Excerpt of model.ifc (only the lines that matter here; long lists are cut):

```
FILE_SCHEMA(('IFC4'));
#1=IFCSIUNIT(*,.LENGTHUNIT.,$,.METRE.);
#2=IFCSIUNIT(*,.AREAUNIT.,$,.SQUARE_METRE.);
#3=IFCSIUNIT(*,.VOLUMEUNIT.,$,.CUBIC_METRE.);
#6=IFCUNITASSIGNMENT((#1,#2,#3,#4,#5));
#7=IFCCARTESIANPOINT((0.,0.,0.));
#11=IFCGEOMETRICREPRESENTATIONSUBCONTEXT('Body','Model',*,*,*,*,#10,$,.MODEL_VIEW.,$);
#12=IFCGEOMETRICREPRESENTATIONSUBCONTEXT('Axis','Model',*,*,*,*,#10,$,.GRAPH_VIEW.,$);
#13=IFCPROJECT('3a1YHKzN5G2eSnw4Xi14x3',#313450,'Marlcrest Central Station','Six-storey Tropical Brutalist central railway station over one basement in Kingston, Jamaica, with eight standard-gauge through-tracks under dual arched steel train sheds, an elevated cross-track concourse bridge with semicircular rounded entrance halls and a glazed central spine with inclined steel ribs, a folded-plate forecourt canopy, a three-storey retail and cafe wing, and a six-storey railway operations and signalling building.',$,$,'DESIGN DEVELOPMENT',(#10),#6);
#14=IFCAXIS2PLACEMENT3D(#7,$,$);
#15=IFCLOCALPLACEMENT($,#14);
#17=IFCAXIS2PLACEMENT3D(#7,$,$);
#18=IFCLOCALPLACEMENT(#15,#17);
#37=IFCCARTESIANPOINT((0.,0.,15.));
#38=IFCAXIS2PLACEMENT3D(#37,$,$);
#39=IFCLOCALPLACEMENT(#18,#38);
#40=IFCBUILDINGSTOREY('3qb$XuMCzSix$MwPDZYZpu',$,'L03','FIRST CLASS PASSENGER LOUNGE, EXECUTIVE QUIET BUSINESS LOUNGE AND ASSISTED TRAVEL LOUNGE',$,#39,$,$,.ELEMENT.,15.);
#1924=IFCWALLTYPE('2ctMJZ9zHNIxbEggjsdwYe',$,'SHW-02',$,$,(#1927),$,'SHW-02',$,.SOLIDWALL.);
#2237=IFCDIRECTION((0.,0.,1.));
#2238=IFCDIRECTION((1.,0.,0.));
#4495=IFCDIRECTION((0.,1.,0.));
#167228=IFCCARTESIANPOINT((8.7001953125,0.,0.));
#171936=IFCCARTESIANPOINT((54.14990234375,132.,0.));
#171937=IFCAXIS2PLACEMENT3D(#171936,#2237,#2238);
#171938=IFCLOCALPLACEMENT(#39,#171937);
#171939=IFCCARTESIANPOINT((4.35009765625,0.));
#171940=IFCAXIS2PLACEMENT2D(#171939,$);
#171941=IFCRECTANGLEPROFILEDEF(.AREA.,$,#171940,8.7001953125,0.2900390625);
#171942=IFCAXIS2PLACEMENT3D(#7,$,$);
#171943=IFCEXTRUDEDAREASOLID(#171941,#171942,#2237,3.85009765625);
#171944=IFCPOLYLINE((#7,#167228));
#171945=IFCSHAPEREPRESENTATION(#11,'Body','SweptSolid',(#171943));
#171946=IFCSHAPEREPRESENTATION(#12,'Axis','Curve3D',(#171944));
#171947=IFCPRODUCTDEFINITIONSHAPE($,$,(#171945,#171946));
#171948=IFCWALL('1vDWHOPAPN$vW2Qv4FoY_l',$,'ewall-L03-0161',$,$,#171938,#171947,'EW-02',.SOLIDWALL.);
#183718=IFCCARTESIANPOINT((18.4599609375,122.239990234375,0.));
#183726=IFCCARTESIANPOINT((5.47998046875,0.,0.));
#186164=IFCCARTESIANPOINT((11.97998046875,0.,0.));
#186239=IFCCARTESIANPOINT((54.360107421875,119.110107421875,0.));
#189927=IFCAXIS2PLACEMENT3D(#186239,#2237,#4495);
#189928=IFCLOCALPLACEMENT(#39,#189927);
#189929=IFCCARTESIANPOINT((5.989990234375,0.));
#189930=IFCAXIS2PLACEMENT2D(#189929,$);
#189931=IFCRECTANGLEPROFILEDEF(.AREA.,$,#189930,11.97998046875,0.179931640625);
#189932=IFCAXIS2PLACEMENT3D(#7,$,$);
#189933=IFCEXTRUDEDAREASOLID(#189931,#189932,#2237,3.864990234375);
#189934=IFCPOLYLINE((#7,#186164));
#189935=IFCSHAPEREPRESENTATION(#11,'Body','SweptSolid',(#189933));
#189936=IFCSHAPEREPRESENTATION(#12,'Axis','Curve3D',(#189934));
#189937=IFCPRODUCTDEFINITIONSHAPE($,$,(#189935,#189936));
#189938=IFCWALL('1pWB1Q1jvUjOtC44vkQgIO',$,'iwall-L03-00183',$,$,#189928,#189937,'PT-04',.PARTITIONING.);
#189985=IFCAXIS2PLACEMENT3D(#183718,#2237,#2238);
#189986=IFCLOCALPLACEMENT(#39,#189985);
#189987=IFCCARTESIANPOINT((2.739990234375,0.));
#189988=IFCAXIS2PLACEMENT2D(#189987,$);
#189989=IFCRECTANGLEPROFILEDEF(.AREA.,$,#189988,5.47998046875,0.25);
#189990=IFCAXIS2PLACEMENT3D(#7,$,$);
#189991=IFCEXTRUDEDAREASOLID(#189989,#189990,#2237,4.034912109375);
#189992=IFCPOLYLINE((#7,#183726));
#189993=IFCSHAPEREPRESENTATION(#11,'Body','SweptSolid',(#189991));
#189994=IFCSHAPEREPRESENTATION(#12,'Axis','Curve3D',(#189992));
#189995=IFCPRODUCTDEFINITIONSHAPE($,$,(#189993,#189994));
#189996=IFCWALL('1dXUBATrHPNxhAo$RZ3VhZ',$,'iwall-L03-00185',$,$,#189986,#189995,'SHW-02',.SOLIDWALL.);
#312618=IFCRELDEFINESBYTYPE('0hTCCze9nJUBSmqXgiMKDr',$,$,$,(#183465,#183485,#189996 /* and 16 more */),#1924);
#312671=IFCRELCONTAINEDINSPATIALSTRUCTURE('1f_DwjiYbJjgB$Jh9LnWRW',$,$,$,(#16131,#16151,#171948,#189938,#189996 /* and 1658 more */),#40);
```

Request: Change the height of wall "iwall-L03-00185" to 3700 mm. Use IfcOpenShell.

```python
import ifcopenshell
import ifcopenshell.geom
import ifcopenshell.util.representation
import ifcopenshell.util.shape
import ifcopenshell.util.unit

model = ifcopenshell.open("model.ifc")
unit_scale = ifcopenshell.util.unit.calculate_unit_scale(model)
settings = ifcopenshell.geom.settings()


def volume(element):
    """Net volume in cubic metres, openings subtracted."""
    shape = ifcopenshell.geom.create_shape(settings, element)
    return ifcopenshell.util.shape.get_volume(shape.geometry)


wall = model.by_guid("1dXUBATrHPNxhAo$RZ3VhZ")
before = volume(wall)

body = ifcopenshell.util.representation.get_representation(wall, "Model", "Body")
solid = body.Items[0]
old_height = solid.Depth
solid.Depth = 3.7 / unit_scale
after = volume(wall)

print(f"height {old_height:g} -> {solid.Depth:g}, volume {before:.3f} -> {after:.3f} m3")

model.write("model_v2.ifc")
```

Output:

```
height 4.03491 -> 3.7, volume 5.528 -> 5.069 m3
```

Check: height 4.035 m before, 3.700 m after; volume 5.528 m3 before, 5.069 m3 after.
